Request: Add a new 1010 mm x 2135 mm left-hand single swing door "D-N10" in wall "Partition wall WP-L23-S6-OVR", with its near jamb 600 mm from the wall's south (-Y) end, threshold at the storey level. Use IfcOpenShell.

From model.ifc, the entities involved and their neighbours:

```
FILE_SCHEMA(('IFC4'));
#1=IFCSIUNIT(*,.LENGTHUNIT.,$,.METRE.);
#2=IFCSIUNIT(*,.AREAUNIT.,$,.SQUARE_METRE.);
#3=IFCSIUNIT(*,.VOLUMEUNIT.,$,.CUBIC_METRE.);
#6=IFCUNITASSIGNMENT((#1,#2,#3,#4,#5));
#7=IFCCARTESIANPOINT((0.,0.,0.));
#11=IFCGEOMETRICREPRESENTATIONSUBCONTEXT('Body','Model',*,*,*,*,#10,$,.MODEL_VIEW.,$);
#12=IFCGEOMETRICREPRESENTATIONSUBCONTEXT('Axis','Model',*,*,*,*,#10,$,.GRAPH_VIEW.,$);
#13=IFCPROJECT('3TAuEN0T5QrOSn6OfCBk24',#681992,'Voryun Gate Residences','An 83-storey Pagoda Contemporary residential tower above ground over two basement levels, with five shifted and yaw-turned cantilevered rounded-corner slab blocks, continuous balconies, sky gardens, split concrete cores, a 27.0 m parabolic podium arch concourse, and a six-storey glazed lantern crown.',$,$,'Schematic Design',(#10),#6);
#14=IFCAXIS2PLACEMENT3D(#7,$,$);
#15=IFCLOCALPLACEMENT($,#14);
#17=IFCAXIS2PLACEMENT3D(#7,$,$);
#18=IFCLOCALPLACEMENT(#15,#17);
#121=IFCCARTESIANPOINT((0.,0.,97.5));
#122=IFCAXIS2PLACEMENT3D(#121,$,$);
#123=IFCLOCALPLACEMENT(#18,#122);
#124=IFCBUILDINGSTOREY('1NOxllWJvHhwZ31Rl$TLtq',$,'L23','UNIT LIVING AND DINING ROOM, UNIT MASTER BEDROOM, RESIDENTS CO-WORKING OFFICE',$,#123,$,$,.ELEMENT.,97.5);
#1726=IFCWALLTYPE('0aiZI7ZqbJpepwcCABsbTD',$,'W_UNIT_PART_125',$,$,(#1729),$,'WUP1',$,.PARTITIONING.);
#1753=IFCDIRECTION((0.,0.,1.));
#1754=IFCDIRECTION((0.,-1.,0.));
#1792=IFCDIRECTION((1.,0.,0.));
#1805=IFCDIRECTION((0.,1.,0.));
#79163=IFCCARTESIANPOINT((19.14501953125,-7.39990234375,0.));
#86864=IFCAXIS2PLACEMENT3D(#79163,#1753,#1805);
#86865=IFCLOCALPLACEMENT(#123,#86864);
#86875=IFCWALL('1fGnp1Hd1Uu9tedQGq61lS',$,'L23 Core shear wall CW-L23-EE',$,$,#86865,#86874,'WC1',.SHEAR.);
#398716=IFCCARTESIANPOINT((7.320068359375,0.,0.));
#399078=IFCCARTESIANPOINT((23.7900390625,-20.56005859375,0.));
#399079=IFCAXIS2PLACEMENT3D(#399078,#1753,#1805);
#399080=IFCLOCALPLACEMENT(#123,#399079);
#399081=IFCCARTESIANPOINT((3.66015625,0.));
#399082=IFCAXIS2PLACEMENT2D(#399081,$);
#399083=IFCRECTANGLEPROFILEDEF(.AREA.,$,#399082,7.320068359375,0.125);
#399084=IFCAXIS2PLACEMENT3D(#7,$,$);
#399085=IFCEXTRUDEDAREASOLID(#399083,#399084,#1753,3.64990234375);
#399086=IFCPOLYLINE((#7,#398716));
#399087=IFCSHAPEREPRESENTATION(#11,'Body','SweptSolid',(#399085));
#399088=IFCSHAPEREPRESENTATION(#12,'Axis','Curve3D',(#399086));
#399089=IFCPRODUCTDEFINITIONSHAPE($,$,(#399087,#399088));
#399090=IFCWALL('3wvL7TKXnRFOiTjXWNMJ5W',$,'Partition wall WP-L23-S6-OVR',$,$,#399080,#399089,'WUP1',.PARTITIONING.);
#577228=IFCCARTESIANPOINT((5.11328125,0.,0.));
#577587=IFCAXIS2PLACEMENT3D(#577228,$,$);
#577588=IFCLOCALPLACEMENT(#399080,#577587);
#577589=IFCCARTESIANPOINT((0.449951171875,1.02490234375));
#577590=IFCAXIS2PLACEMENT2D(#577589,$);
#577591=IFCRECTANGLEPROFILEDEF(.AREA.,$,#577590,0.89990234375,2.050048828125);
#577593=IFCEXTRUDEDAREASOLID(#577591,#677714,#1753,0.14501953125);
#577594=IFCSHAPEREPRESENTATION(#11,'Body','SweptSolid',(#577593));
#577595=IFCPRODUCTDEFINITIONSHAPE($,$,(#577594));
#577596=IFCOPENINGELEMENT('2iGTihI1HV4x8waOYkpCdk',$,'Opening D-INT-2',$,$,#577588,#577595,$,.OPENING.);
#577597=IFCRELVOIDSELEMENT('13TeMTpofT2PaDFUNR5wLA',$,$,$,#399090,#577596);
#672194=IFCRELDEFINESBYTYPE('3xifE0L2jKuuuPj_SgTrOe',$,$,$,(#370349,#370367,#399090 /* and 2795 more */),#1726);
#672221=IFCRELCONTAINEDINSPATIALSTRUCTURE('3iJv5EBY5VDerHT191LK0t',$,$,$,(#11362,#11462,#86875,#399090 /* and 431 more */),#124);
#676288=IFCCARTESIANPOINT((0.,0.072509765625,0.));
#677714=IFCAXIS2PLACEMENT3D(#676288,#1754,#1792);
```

```python
import numpy as np
import ifcopenshell
import ifcopenshell.api.feature
import ifcopenshell.api.geometry
import ifcopenshell.api.root
import ifcopenshell.api.spatial
import ifcopenshell.geom
import ifcopenshell.util.element
import ifcopenshell.util.placement
import ifcopenshell.util.representation
import ifcopenshell.util.shape
import ifcopenshell.util.unit

model = ifcopenshell.open("model.ifc")
unit_scale = ifcopenshell.util.unit.calculate_unit_scale(model)
settings = ifcopenshell.geom.settings()


def volume(element):
    """Net volume in cubic metres, openings subtracted."""
    shape = ifcopenshell.geom.create_shape(settings, element)
    return ifcopenshell.util.shape.get_volume(shape.geometry)


wall = model.by_guid("3wvL7TKXnRFOiTjXWNMJ5W")
storey = ifcopenshell.util.element.get_container(wall, ifc_class="IfcBuildingStorey")
context = ifcopenshell.util.representation.get_context(model, "Model", "Body", "MODEL_VIEW")
before = volume(wall)

width, height, from_end, sill = 1.01, 2.135, 0.6, 0.0  # metres

# The wall runs along its own X axis, and the end named is its -X end.
wall_shape = ifcopenshell.geom.create_shape(settings, wall)
x, y, z = ifcopenshell.util.shape.get_vertices(wall_shape.geometry).T
start = x.min() + from_end
face, thickness = float(y.min()), float(y.max() - y.min())
wall_matrix = ifcopenshell.util.placement.get_local_placement(wall.ObjectPlacement)
level = ifcopenshell.util.placement.get_local_placement(storey.ObjectPlacement)[2, 3]


def in_wall(x, y):
    """Placement at x, y metres in the wall's axes, at sill height."""
    matrix = wall_matrix.copy()
    matrix[:, 3] = wall_matrix @ np.array([x / unit_scale, y / unit_scale, 0.0, 1.0])
    matrix[2, 3] = level + sill / unit_scale
    return matrix


# Opening: a box that overshoots both wall faces by 50 mm.
opening = ifcopenshell.api.root.create_entity(model, ifc_class="IfcOpeningElement", predefined_type="OPENING")
box = ifcopenshell.api.geometry.add_wall_representation(
    model, context=context, length=width, height=height, thickness=thickness + 0.1
)
ifcopenshell.api.geometry.assign_representation(model, product=opening, representation=box)
ifcopenshell.api.geometry.edit_object_placement(model, product=opening, matrix=in_wall(start, face - 0.05), is_si=False)
ifcopenshell.api.feature.add_feature(model, feature=opening, element=wall)

door = ifcopenshell.api.root.create_entity(model, ifc_class="IfcDoor", name="D-N10", predefined_type="DOOR")
door.OverallWidth, door.OverallHeight = width / unit_scale, height / unit_scale
door.OperationType = "SINGLE_SWING_LEFT"
body = ifcopenshell.api.geometry.add_door_representation(
    model,
    context=context,
    overall_width=door.OverallWidth,
    overall_height=door.OverallHeight,
    operation_type="SINGLE_SWING_LEFT",
    lining_properties={"LiningDepth": thickness / unit_scale, "ThresholdDepth": thickness / unit_scale},
)
ifcopenshell.api.geometry.assign_representation(model, product=door, representation=body)
ifcopenshell.api.spatial.assign_container(model, products=[door], relating_structure=storey)
ifcopenshell.api.feature.add_filling(model, opening=opening, element=door)

# The lining spans the wall, so the door starts at the wall face.
ifcopenshell.api.geometry.edit_object_placement(model, product=door, matrix=in_wall(start, face), is_si=False)

after = volume(wall)

print(f"wall volume {before:.3f} -> {after:.3f} m3")

model.write("model-out.ifc")
```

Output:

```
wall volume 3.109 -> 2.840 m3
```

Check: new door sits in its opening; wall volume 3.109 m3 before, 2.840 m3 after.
